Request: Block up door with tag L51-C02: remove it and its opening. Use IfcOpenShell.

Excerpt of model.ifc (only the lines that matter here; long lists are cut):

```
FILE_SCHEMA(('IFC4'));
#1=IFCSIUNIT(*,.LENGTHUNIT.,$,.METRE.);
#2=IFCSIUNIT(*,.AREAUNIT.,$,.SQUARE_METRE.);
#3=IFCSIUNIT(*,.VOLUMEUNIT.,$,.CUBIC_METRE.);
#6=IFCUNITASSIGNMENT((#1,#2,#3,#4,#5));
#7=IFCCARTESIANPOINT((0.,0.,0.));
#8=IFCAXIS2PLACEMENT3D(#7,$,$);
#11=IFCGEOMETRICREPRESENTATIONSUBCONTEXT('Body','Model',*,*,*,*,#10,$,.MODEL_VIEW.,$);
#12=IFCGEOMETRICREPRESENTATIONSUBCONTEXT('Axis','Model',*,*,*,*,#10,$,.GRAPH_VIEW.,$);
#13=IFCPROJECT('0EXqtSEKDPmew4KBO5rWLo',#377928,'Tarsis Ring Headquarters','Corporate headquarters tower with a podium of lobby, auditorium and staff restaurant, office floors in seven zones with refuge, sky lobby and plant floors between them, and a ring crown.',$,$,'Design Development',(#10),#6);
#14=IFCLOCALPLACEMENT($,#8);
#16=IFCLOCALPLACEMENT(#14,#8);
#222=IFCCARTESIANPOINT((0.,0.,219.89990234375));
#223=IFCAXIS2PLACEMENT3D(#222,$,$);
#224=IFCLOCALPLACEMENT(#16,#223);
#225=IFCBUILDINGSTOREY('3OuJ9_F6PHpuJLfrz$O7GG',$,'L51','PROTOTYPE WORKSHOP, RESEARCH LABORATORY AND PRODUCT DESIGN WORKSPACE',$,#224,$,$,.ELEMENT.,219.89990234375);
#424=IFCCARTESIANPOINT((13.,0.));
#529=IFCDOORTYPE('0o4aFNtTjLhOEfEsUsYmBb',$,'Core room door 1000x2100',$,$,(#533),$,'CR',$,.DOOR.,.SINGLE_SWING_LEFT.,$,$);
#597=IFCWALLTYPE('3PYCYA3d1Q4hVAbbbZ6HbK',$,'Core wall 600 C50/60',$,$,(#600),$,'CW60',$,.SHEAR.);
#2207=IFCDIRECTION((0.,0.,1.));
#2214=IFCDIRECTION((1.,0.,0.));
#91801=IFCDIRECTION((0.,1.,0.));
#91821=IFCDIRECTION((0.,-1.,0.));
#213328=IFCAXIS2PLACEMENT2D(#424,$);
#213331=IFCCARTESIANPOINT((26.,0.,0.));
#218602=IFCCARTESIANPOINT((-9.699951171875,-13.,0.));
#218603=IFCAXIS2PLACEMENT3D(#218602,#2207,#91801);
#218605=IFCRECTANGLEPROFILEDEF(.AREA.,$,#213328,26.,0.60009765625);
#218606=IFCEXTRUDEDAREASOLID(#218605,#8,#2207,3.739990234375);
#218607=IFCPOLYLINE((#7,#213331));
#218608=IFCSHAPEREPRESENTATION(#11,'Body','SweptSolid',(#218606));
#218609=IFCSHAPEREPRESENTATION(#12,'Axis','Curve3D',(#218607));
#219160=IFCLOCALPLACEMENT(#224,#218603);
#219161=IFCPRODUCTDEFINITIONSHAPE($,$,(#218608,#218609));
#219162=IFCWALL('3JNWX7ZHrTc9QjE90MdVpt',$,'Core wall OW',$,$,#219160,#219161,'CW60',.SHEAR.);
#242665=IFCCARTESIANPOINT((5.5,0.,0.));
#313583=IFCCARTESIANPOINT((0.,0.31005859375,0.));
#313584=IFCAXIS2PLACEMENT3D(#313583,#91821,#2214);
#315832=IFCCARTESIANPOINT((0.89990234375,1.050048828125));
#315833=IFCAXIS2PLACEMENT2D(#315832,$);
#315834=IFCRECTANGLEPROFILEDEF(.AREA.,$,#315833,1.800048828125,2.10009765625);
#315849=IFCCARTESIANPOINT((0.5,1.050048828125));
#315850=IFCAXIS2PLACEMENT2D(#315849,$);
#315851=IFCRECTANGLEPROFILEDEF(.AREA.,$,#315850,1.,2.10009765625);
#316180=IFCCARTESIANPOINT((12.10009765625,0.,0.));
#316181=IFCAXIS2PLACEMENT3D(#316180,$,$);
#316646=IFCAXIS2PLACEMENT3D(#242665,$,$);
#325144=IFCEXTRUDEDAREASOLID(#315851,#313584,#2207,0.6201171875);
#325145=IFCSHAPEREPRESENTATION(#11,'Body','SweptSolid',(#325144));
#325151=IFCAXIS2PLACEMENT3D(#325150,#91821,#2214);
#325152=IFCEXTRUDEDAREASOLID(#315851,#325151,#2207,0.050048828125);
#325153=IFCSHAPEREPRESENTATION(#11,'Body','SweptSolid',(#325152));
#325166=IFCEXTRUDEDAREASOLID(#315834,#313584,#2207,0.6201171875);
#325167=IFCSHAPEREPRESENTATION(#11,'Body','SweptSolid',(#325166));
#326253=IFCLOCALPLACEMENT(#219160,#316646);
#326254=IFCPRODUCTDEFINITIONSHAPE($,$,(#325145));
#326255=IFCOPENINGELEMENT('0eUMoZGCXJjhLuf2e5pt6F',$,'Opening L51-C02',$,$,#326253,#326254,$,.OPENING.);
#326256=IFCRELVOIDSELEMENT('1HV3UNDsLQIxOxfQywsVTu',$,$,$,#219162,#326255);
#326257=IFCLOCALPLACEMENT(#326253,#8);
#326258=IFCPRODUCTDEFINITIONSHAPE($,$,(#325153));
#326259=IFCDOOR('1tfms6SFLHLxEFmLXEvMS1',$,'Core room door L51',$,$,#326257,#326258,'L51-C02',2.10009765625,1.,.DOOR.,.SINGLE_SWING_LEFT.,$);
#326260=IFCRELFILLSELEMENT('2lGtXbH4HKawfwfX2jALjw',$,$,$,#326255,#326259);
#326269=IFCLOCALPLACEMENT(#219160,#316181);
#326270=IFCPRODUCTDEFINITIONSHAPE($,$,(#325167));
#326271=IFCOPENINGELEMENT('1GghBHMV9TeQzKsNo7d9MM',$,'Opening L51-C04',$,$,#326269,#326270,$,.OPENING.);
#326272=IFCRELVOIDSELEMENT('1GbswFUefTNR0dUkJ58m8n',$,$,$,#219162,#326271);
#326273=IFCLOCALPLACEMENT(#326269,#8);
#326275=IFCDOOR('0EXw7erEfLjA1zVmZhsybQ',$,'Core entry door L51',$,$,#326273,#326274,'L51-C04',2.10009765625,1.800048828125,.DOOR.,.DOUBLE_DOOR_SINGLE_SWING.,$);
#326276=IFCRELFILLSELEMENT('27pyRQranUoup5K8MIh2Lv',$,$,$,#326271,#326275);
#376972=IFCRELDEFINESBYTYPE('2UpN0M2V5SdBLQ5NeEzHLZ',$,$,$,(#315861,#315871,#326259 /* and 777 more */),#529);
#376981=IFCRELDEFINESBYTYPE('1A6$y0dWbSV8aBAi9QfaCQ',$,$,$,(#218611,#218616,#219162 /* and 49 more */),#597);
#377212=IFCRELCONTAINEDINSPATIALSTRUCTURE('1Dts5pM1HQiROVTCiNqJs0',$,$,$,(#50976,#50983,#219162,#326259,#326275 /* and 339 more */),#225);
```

```python
import ifcopenshell
import ifcopenshell.api.feature
import ifcopenshell.api.root
import ifcopenshell.geom
import ifcopenshell.util.shape

model = ifcopenshell.open("model.ifc")
settings = ifcopenshell.geom.settings()


def volume(element):
    """Net volume in cubic metres, openings subtracted."""
    shape = ifcopenshell.geom.create_shape(settings, element)
    return ifcopenshell.util.shape.get_volume(shape.geometry)


door = model.by_id(326259)
opening = door.FillsVoids[0].RelatingOpeningElement
wall = opening.VoidsElements[0].RelatingBuildingElement
before = volume(wall)

ifcopenshell.api.root.remove_product(model, product=door)
ifcopenshell.api.feature.remove_feature(model, feature=opening)

after = volume(wall)

print(f"wall volume {before:.3f} -> {after:.3f} m3")

model.write("model_updated.ifc")
```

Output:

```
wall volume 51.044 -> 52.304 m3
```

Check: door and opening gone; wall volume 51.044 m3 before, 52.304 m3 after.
